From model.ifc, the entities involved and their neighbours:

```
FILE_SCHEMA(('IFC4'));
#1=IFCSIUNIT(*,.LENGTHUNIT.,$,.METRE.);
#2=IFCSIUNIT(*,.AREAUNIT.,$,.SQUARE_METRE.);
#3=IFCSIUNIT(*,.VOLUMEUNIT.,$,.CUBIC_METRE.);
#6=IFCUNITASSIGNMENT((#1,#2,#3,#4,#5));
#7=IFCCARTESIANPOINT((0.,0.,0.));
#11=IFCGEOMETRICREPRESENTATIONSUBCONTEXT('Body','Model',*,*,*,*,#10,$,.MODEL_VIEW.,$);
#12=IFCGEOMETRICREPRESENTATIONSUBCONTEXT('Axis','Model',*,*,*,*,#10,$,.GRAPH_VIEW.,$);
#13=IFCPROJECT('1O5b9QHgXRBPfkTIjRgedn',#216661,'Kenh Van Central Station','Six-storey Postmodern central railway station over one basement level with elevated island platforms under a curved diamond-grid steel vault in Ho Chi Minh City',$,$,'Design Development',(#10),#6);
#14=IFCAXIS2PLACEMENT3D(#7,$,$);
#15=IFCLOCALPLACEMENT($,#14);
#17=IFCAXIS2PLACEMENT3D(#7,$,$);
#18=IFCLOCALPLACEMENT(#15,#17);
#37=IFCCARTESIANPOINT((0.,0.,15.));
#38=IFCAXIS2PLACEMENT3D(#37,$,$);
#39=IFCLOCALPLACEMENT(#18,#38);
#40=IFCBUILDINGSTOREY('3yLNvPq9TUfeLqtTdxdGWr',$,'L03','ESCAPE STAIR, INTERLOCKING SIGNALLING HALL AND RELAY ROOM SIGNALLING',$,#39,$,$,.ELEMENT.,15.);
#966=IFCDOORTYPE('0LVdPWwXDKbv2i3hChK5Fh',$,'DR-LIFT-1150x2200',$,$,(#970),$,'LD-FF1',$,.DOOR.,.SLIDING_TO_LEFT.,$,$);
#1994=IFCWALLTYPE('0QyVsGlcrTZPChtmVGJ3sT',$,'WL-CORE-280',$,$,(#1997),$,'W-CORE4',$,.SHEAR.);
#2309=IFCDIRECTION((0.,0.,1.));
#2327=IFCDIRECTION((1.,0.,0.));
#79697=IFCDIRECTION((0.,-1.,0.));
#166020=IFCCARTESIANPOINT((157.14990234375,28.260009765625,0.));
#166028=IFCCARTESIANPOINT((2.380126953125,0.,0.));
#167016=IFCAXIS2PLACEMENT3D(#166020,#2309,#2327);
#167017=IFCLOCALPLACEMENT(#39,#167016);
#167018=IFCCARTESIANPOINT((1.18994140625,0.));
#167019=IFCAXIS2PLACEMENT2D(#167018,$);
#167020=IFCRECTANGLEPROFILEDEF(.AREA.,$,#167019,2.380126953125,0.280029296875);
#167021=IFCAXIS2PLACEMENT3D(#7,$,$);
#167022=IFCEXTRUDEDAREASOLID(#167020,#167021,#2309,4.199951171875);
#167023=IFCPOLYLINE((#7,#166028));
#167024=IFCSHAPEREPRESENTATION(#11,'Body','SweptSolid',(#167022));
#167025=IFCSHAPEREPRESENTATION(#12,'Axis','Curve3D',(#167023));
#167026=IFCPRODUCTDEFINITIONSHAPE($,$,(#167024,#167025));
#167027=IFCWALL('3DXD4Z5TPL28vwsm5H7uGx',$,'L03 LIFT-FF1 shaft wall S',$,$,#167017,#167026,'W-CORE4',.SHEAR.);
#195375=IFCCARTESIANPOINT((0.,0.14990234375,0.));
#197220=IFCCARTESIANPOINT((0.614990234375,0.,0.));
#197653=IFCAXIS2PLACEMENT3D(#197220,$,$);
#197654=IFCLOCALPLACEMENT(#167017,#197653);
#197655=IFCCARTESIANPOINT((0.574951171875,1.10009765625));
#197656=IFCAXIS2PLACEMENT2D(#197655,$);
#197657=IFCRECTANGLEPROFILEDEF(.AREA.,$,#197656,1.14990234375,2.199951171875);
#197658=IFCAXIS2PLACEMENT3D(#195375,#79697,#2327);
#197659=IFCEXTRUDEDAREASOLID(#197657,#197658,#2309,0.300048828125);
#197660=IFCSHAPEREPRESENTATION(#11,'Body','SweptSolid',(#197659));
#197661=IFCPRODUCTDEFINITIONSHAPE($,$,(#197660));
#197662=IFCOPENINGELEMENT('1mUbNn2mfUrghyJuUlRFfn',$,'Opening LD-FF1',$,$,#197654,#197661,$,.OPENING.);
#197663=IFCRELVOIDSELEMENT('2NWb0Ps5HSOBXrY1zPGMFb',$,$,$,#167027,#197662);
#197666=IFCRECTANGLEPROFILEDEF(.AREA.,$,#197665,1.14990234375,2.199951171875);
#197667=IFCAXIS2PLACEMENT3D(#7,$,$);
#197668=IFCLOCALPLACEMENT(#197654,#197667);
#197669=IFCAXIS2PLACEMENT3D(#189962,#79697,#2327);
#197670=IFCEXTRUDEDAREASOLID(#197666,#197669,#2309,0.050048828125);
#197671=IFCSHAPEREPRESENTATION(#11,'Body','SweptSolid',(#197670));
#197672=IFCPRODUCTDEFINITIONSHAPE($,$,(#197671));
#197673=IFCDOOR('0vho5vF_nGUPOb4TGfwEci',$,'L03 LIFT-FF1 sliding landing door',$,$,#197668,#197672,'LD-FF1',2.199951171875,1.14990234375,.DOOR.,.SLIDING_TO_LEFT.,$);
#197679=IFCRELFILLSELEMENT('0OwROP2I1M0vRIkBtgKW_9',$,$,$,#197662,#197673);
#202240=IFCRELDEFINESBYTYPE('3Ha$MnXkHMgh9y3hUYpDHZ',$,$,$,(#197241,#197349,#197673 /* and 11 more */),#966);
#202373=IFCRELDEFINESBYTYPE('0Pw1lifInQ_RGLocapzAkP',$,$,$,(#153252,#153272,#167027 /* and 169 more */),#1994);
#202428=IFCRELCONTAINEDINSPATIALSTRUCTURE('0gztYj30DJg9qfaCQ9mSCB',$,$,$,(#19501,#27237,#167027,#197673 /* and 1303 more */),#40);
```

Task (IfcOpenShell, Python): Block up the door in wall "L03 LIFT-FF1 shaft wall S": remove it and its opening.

```python
import ifcopenshell
import ifcopenshell.api.feature
import ifcopenshell.api.root
import ifcopenshell.geom
import ifcopenshell.util.shape

model = ifcopenshell.open("model.ifc")
settings = ifcopenshell.geom.settings()


def volume(element):
    """Net volume in cubic metres, openings subtracted."""
    shape = ifcopenshell.geom.create_shape(settings, element)
    return ifcopenshell.util.shape.get_volume(shape.geometry)


door = model.by_guid("0vho5vF_nGUPOb4TGfwEci")
opening = door.FillsVoids[0].RelatingOpeningElement
wall = opening.VoidsElements[0].RelatingBuildingElement
before = volume(wall)

ifcopenshell.api.root.remove_product(model, product=door)
ifcopenshell.api.feature.remove_feature(model, feature=opening)

after = volume(wall)

print(f"wall volume {before:.3f} -> {after:.3f} m3")

model.write("model_updated.ifc")
```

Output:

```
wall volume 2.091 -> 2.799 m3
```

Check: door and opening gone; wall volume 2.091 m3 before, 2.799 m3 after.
